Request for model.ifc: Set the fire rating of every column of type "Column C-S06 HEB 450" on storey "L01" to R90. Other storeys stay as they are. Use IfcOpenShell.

First a look at what the model holds.

```python
import ifcopenshell
import ifcopenshell.util.element

model = ifcopenshell.open("model.ifc")
print(model.schema)
storey = next(s for s in model.by_type("IfcBuildingStorey") if s.Name == "L01")
columns = [e for e in ifcopenshell.util.element.get_decomposition(storey) if e.is_a("IfcColumn")]
seen = {}
for e in columns:
    element_type = ifcopenshell.util.element.get_type(e)
    key = (element_type.Name if element_type != e and element_type else None, ifcopenshell.util.element.get_pset(e, "Pset_ColumnCommon", "FireRating"))
    seen[key] = seen.get(key, 0) + 1
for (name, value), count in sorted(seen.items(), key=str):
    print(count, "x", name, "|", value)
```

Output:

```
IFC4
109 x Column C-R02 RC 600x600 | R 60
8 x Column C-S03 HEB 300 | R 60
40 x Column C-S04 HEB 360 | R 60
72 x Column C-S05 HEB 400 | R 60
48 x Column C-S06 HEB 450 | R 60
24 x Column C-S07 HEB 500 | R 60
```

```python
import ifcopenshell
import ifcopenshell.api.pset
import ifcopenshell.util.element

model = ifcopenshell.open("model.ifc")

storey = next(s for s in model.by_type("IfcBuildingStorey") if s.Name == "L01")
columns = [e for e in ifcopenshell.util.element.get_decomposition(storey) if e.is_a("IfcColumn")]

count = 0
for e in columns:
    element_type = ifcopenshell.util.element.get_type(e)
    if element_type in (None, e) or element_type.Name != "Column C-S06 HEB 450":
        continue
    # add_pset returns the element's existing set when there is one.
    pset = ifcopenshell.api.pset.add_pset(model, product=e, name="Pset_ColumnCommon")
    ifcopenshell.api.pset.edit_pset(model, pset=pset, properties={"FireRating": "R90"})
    count += 1

print(count, "columns updated")

model.write("model_v2.ifc")
```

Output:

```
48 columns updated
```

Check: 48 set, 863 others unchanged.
